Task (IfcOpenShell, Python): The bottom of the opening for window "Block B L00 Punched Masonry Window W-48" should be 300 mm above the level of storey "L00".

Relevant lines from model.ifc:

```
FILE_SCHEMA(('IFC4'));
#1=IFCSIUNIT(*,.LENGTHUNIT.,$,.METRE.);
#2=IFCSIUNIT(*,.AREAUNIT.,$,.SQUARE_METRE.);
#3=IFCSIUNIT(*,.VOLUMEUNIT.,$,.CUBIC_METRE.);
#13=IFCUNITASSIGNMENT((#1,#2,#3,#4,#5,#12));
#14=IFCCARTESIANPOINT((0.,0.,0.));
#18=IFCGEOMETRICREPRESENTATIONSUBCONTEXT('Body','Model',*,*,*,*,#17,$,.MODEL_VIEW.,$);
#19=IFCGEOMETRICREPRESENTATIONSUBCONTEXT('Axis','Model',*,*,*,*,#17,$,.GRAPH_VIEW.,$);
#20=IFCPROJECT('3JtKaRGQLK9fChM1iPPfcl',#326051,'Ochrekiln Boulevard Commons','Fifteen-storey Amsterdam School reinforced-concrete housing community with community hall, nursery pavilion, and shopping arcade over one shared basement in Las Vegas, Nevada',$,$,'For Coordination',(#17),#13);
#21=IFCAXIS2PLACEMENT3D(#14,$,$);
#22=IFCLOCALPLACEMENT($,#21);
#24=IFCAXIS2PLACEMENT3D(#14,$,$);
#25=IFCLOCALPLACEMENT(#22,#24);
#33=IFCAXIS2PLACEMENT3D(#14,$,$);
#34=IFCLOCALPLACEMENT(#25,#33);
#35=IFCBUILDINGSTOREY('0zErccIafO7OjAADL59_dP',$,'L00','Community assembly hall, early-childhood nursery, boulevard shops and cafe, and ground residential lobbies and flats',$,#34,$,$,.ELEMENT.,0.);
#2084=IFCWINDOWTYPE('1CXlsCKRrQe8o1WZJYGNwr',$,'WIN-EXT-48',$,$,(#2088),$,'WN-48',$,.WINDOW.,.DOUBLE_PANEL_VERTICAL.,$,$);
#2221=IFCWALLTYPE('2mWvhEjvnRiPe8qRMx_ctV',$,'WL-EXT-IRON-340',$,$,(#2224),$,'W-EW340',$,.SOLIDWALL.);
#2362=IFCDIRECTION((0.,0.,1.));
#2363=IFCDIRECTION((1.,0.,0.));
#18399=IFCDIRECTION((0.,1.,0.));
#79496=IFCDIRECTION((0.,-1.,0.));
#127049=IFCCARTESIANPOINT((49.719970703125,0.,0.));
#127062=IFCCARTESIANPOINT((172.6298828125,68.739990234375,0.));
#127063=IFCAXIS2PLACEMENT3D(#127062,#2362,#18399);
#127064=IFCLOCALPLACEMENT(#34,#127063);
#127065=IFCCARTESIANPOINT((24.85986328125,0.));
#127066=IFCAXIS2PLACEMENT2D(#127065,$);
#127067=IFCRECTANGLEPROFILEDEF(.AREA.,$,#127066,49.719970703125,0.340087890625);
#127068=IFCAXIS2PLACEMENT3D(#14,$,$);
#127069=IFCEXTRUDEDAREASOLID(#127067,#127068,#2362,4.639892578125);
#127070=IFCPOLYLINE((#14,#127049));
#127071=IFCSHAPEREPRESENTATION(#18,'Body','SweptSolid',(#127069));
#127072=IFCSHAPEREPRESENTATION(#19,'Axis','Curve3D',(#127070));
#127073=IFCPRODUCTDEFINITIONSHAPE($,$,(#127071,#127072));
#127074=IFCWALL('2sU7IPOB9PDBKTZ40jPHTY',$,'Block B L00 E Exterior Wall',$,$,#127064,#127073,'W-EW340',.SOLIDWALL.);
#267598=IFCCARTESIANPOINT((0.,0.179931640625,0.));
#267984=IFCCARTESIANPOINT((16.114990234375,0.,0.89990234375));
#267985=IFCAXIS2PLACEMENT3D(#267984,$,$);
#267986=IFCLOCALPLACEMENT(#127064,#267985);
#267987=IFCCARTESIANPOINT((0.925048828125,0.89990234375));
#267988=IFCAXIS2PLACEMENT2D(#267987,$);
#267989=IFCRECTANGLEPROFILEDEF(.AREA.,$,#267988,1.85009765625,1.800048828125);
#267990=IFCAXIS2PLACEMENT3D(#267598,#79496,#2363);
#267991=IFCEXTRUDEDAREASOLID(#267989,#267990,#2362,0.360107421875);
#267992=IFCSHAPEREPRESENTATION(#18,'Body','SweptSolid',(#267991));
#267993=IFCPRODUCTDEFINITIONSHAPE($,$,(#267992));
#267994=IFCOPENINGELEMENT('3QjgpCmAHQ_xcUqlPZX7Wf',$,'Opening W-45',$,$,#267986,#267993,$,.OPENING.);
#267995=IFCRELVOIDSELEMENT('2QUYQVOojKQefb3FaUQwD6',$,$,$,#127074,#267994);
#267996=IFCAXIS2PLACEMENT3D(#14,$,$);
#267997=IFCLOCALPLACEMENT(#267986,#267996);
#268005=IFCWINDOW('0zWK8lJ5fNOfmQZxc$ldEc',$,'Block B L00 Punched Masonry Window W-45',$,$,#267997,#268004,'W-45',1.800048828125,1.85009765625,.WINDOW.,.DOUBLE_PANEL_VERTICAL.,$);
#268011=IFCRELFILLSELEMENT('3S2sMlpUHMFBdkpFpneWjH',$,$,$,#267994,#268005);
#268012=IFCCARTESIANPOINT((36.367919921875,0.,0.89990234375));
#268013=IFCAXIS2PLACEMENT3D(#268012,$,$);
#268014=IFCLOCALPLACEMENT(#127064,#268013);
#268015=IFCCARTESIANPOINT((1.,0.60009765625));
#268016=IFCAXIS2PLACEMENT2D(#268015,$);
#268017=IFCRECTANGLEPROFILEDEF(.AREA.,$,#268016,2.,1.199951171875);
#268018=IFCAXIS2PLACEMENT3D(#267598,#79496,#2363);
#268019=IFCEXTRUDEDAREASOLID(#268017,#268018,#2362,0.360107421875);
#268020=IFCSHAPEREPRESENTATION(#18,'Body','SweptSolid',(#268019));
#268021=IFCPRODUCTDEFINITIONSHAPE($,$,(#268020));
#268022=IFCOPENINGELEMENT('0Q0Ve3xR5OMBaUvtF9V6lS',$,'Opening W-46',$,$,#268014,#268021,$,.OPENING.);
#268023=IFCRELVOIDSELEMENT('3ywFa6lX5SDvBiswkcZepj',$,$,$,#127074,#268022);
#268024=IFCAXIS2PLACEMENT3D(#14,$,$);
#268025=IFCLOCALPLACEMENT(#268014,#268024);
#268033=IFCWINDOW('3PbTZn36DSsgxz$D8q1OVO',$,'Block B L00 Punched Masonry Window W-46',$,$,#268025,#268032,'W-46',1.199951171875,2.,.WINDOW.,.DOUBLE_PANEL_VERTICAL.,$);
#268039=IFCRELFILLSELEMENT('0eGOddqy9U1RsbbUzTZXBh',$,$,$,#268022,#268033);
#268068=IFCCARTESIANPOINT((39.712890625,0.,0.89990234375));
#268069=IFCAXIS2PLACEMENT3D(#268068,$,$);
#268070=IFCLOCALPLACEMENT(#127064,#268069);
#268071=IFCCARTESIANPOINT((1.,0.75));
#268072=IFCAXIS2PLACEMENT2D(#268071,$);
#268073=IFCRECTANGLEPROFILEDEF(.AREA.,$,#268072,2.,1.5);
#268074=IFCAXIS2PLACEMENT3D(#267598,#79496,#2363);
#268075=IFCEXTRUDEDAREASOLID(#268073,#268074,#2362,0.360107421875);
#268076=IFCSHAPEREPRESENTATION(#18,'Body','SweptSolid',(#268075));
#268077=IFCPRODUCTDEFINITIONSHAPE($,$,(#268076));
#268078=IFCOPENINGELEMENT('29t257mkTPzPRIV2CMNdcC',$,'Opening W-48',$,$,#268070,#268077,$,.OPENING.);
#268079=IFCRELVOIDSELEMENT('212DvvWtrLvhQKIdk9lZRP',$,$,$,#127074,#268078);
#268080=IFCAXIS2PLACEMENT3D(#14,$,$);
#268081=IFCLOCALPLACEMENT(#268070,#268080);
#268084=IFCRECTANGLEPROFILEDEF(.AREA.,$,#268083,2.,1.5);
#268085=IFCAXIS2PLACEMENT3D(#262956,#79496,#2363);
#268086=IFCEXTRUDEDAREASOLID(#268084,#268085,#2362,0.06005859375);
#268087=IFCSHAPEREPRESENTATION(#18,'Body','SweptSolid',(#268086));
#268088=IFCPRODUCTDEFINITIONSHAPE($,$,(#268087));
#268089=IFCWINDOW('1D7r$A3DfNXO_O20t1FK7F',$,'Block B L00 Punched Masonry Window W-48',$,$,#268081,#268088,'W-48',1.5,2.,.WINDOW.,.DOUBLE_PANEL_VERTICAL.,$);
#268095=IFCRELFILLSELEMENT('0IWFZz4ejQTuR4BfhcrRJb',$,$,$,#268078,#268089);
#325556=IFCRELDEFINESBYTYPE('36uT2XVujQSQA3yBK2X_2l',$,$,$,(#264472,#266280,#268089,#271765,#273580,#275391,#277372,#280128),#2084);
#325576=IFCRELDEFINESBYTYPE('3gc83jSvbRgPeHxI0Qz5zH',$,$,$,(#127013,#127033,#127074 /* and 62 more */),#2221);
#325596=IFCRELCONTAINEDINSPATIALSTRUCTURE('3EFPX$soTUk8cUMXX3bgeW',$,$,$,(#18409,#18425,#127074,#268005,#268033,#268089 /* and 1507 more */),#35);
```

```python
import numpy as np
import ifcopenshell
import ifcopenshell.api.geometry
import ifcopenshell.geom
import ifcopenshell.util.element
import ifcopenshell.util.placement
import ifcopenshell.util.shape
import ifcopenshell.util.unit

model = ifcopenshell.open("model.ifc")
unit_scale = ifcopenshell.util.unit.calculate_unit_scale(model)

window = model.by_guid("1D7r$A3DfNXO_O20t1FK7F")
opening = window.FillsVoids[0].RelatingOpeningElement
storey = ifcopenshell.util.element.get_container(window, ifc_class="IfcBuildingStorey")
level = ifcopenshell.util.placement.get_local_placement(storey.ObjectPlacement)[2, 3]

# The opening's origin need not be at the sill, so measure its lowest point.
shape = ifcopenshell.geom.create_shape(ifcopenshell.geom.settings(), opening)
bottom = ifcopenshell.util.shape.get_shape_bottom_elevation(shape, shape.geometry) / unit_scale
dz = level + 0.3 / unit_scale - bottom

shift = np.array([0.0, 0.0, dz])
# The window is placed relative to its opening, so it follows when the opening moves.
matrix = ifcopenshell.util.placement.get_local_placement(opening.ObjectPlacement)
matrix[:3, 3] += shift
ifcopenshell.api.geometry.edit_object_placement(
    model, product=opening, matrix=matrix, is_si=False, should_transform_children=True
)

print(f"moved by {dz * unit_scale:+.3f} m")

model.write("model_updated.ifc")
```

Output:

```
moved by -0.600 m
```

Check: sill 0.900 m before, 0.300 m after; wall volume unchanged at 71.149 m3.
